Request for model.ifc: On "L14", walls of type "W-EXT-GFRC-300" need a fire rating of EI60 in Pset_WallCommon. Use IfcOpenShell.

First a look at what the model holds.

```python
import ifcopenshell
import ifcopenshell.util.element

model = ifcopenshell.open("model.ifc")
print(model.schema)
storey = next(s for s in model.by_type("IfcBuildingStorey") if s.Name == "L14")
walls = [e for e in ifcopenshell.util.element.get_decomposition(storey) if e.is_a("IfcWall")]
seen = {}
for e in walls:
    element_type = ifcopenshell.util.element.get_type(e)
    key = (element_type.Name if element_type != e and element_type else None, ifcopenshell.util.element.get_pset(e, "Pset_WallCommon", "FireRating"))
    seen[key] = seen.get(key, 0) + 1
for (name, value), count in sorted(seen.items(), key=str):
    print(count, "x", name, "|", value)
```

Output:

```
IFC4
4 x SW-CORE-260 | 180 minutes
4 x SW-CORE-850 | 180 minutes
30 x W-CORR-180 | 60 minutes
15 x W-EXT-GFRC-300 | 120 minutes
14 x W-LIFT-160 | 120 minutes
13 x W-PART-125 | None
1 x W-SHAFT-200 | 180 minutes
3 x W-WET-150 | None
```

```python
import ifcopenshell
import ifcopenshell.api.pset
import ifcopenshell.util.element

model = ifcopenshell.open("model.ifc")

storey = next(s for s in model.by_type("IfcBuildingStorey") if s.Name == "L14")
walls = [e for e in ifcopenshell.util.element.get_decomposition(storey) if e.is_a("IfcWall")]

count = 0
for e in walls:
    element_type = ifcopenshell.util.element.get_type(e)
    if element_type in (None, e) or element_type.Name != "W-EXT-GFRC-300":
        continue
    found = ifcopenshell.util.element.get_pset(e, "Pset_WallCommon", should_inherit=False)
    if found:
        pset = model.by_id(found["id"])
        if len(ifcopenshell.util.element.get_elements_by_pset(pset)) > 1:
            pset = ifcopenshell.api.pset.unshare_pset(model, products=[e], pset=pset)[0]
    else:
        pset = ifcopenshell.api.pset.add_pset(model, product=e, name="Pset_WallCommon")
    ifcopenshell.api.pset.edit_pset(model, pset=pset, properties={"FireRating": "EI60"})
    count += 1

print(count, "walls updated")

model.write("model_v2.ifc")
```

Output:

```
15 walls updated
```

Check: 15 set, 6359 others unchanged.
